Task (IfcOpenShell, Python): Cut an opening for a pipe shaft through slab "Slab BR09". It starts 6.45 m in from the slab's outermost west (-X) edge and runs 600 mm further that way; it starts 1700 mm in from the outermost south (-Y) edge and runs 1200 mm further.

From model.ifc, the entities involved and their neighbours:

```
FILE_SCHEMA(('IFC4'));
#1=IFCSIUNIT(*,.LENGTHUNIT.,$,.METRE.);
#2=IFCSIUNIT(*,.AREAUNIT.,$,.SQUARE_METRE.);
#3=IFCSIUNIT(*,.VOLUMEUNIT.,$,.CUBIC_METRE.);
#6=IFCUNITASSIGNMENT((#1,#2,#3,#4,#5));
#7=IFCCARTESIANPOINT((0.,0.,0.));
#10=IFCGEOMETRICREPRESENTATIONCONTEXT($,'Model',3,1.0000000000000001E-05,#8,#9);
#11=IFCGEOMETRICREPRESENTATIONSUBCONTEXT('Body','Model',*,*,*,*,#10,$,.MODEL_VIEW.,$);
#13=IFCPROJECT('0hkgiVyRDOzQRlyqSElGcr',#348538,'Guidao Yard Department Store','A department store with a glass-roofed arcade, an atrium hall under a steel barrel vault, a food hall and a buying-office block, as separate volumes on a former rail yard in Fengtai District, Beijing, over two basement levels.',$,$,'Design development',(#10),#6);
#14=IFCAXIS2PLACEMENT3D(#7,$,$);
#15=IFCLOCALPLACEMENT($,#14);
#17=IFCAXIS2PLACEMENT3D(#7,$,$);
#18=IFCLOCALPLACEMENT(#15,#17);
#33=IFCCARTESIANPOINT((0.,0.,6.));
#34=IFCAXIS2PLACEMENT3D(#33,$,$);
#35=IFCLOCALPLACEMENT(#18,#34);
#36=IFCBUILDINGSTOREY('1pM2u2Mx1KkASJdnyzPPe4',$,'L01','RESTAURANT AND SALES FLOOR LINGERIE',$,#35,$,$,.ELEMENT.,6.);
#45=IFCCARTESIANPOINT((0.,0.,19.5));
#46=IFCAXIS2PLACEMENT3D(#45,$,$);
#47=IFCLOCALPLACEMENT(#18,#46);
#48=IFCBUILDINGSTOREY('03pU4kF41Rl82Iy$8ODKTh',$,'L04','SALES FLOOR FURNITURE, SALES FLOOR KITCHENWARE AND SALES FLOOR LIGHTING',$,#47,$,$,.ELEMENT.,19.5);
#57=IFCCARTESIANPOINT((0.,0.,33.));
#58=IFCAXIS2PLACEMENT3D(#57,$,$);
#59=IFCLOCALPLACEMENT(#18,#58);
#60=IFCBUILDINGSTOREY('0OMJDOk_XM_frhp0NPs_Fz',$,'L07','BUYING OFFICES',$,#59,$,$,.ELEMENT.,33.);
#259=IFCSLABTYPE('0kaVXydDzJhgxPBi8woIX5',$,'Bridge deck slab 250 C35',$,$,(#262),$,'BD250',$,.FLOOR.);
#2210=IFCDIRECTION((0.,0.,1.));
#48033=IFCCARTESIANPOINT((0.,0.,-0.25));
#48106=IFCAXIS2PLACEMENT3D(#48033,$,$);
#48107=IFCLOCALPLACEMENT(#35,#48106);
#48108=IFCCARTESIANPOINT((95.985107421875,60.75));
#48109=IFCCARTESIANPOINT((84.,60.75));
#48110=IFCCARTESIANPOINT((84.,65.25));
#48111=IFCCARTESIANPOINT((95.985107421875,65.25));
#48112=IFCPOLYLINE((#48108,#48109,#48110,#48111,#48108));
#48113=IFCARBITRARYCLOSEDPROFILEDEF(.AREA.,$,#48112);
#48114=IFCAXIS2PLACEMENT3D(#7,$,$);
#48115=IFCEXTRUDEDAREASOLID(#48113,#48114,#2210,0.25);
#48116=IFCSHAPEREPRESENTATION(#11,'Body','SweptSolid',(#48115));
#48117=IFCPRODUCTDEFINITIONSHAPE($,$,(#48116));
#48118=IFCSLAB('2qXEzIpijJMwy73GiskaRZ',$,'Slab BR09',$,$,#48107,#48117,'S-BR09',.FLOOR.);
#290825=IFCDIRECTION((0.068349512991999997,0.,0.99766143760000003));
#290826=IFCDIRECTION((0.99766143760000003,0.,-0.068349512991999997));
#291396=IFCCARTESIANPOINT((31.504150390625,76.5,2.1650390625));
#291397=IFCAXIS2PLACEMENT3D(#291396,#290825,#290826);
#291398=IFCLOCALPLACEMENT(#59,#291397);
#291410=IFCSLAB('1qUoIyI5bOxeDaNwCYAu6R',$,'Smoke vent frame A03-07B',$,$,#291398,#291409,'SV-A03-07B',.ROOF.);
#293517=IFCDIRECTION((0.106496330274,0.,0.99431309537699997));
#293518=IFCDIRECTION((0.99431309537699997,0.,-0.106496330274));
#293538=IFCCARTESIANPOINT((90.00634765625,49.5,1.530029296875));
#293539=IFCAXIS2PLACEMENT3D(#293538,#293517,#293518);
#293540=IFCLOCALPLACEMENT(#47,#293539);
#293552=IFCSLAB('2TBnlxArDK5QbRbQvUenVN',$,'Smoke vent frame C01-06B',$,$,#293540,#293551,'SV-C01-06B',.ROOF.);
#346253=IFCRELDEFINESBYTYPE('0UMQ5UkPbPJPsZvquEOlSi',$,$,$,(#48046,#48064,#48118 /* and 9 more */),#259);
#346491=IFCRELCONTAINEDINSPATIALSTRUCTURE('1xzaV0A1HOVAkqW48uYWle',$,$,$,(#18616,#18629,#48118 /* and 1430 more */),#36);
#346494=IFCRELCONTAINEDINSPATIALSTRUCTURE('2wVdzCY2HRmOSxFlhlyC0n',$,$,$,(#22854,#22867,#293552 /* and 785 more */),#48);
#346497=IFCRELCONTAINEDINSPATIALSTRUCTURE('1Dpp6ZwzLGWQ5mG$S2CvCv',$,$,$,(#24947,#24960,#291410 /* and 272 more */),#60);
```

```python
import numpy as np
import ifcopenshell
import ifcopenshell.api.feature
import ifcopenshell.api.geometry
import ifcopenshell.api.root
import ifcopenshell.geom
import ifcopenshell.util.placement
import ifcopenshell.util.representation
import ifcopenshell.util.shape
import ifcopenshell.util.unit

model = ifcopenshell.open("model.ifc")
unit_scale = ifcopenshell.util.unit.calculate_unit_scale(model)
settings = ifcopenshell.geom.settings()


def volume(element):
    """Net volume in cubic metres, openings subtracted."""
    shape = ifcopenshell.geom.create_shape(settings, element)
    return ifcopenshell.util.shape.get_volume(shape.geometry)


slab = model.by_guid("2qXEzIpijJMwy73GiskaRZ")
before = volume(slab)

# Extent in the slab's own axes, in metres. The edges named are its -X and -Y sides.
slab_shape = ifcopenshell.geom.create_shape(settings, slab)
vertices = ifcopenshell.util.shape.get_vertices(slab_shape.geometry)
x_min, y_min, bottom = vertices.min(axis=0)
top = vertices[:, 2].max()

opening = ifcopenshell.api.root.create_entity(model, ifc_class="IfcOpeningElement", name="Pipe shaft opening", predefined_type="OPENING")
context = ifcopenshell.util.representation.get_context(model, "Model", "Body", "MODEL_VIEW")
width, depth = 0.6, 1.2
outline = [(0.0, 0.0), (width, 0.0), (width, depth), (0.0, depth), (0.0, 0.0)]
# Overshoot both faces by 50 mm so the cut is clean.
shape = ifcopenshell.api.geometry.add_slab_representation(
    model, context=context, depth=top - bottom + 0.1, polyline=outline
)
ifcopenshell.api.geometry.assign_representation(model, product=opening, representation=shape)

matrix = ifcopenshell.util.placement.get_local_placement(slab.ObjectPlacement)
matrix[:, 3] = matrix @ np.append(np.array([x_min + 6.45, y_min + 1.7, bottom - 0.05]) / unit_scale, 1.0)
ifcopenshell.api.geometry.edit_object_placement(model, product=opening, matrix=matrix, is_si=False)
ifcopenshell.api.feature.add_feature(model, feature=opening, element=slab)

after = volume(slab)

print(f"slab volume {before:.3f} -> {after:.3f} m3")

model.write("model_rev.ifc")
```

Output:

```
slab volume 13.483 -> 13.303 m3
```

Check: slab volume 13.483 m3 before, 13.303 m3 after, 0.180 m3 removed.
